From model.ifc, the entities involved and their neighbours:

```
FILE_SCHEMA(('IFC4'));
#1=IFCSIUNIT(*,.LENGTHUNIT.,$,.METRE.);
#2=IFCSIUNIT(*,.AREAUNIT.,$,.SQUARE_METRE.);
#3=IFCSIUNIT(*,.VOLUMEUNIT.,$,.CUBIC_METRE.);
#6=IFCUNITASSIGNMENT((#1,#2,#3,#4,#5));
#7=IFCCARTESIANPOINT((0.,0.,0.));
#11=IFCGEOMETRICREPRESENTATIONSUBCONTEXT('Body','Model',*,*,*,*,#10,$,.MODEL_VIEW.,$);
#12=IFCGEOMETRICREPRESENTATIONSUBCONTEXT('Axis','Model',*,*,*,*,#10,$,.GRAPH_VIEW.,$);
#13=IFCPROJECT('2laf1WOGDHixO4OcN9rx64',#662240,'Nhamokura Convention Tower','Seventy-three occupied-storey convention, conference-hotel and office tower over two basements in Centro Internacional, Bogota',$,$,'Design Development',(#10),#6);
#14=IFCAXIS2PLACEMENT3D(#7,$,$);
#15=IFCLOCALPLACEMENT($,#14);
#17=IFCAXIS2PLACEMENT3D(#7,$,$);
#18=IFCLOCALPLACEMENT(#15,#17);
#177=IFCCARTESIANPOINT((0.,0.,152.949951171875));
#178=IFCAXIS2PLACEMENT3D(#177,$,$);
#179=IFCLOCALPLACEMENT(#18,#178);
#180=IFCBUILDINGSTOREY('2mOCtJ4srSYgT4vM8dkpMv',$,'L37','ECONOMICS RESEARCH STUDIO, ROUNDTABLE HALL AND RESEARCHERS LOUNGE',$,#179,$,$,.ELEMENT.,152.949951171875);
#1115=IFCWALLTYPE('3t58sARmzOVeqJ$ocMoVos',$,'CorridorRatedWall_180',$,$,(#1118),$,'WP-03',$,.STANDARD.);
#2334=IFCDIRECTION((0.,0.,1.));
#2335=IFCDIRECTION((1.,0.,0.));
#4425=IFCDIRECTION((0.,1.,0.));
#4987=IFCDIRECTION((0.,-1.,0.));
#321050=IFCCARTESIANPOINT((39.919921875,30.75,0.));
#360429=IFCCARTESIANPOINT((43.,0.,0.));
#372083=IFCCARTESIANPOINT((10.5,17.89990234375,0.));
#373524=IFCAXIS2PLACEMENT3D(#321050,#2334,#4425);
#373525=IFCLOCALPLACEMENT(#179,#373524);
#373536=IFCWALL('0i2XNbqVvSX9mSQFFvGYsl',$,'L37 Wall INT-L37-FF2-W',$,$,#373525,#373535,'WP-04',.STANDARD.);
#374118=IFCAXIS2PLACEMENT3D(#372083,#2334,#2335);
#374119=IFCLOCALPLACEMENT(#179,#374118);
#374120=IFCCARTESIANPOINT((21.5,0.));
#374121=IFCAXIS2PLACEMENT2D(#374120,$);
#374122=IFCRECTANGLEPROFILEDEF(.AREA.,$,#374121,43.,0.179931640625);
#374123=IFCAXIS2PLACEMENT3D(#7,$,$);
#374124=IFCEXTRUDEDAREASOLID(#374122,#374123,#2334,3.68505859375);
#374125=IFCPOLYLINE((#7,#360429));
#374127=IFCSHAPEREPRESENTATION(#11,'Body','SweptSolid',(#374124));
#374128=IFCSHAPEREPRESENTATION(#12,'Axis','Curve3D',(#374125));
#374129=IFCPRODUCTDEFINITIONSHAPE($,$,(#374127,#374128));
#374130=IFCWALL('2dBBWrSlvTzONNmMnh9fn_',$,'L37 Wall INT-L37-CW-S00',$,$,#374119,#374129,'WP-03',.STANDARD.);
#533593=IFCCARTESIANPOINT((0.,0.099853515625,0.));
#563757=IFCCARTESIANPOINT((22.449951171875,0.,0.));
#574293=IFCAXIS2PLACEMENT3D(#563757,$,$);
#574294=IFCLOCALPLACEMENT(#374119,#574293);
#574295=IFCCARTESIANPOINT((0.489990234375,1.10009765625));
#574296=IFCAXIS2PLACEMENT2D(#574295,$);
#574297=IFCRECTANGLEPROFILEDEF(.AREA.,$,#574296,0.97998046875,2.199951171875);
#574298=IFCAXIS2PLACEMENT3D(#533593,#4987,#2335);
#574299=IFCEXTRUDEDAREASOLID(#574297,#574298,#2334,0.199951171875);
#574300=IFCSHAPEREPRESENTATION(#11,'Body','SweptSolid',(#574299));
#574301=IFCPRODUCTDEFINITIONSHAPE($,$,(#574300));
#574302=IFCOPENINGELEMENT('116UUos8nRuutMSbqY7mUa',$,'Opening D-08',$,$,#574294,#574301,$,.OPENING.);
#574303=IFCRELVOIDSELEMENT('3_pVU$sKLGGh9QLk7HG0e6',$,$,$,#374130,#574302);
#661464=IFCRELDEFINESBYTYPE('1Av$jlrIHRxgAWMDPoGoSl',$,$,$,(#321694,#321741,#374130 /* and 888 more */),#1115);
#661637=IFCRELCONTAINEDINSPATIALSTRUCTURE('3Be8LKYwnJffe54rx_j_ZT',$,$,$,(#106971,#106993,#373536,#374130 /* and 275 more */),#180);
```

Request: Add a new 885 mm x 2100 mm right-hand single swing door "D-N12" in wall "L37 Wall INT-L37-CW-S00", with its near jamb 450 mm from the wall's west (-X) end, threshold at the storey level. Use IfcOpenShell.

```python
import numpy as np
import ifcopenshell
import ifcopenshell.api.feature
import ifcopenshell.api.geometry
import ifcopenshell.api.root
import ifcopenshell.api.spatial
import ifcopenshell.geom
import ifcopenshell.util.element
import ifcopenshell.util.placement
import ifcopenshell.util.representation
import ifcopenshell.util.shape
import ifcopenshell.util.unit

model = ifcopenshell.open("model.ifc")
unit_scale = ifcopenshell.util.unit.calculate_unit_scale(model)
settings = ifcopenshell.geom.settings()


def volume(element):
    """Net volume in cubic metres, openings subtracted."""
    shape = ifcopenshell.geom.create_shape(settings, element)
    return ifcopenshell.util.shape.get_volume(shape.geometry)


wall = model.by_guid("2dBBWrSlvTzONNmMnh9fn_")
storey = ifcopenshell.util.element.get_container(wall, ifc_class="IfcBuildingStorey")
context = ifcopenshell.util.representation.get_context(model, "Model", "Body", "MODEL_VIEW")
before = volume(wall)

width, height, from_end, sill = 0.885, 2.1, 0.45, 0.0  # metres

# The wall runs along its own X axis, and the end named is its -X end.
wall_shape = ifcopenshell.geom.create_shape(settings, wall)
x, y, z = ifcopenshell.util.shape.get_vertices(wall_shape.geometry).T
start = x.min() + from_end
face, thickness = float(y.min()), float(y.max() - y.min())
wall_matrix = ifcopenshell.util.placement.get_local_placement(wall.ObjectPlacement)
level = ifcopenshell.util.placement.get_local_placement(storey.ObjectPlacement)[2, 3]


def in_wall(x, y):
    """Placement at x, y metres in the wall's axes, at sill height."""
    matrix = wall_matrix.copy()
    matrix[:, 3] = wall_matrix @ np.array([x / unit_scale, y / unit_scale, 0.0, 1.0])
    matrix[2, 3] = level + sill / unit_scale
    return matrix


# Opening: a box that overshoots both wall faces by 50 mm.
opening = ifcopenshell.api.root.create_entity(model, ifc_class="IfcOpeningElement", predefined_type="OPENING")
box = ifcopenshell.api.geometry.add_wall_representation(
    model, context=context, length=width, height=height, thickness=thickness + 0.1
)
ifcopenshell.api.geometry.assign_representation(model, product=opening, representation=box)
ifcopenshell.api.geometry.edit_object_placement(model, product=opening, matrix=in_wall(start, face - 0.05), is_si=False)
ifcopenshell.api.feature.add_feature(model, feature=opening, element=wall)

door = ifcopenshell.api.root.create_entity(model, ifc_class="IfcDoor", name="D-N12", predefined_type="DOOR")
door.OverallWidth, door.OverallHeight = width / unit_scale, height / unit_scale
door.OperationType = "SINGLE_SWING_RIGHT"
body = ifcopenshell.api.geometry.add_door_representation(
    model,
    context=context,
    overall_width=door.OverallWidth,
    overall_height=door.OverallHeight,
    operation_type="SINGLE_SWING_RIGHT",
    lining_properties={"LiningDepth": thickness / unit_scale, "ThresholdDepth": thickness / unit_scale},
)
ifcopenshell.api.geometry.assign_representation(model, product=door, representation=body)
ifcopenshell.api.spatial.assign_container(model, products=[door], relating_structure=storey)
ifcopenshell.api.feature.add_filling(model, opening=opening, element=door)

# The lining spans the wall, so the door starts at the wall face.
ifcopenshell.api.geometry.edit_object_placement(model, product=door, matrix=in_wall(start, face), is_si=False)

after = volume(wall)

print(f"wall volume {before:.3f} -> {after:.3f} m3")

model.write("model_updated.ifc")
```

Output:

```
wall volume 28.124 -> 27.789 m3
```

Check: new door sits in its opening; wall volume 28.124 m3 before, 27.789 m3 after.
